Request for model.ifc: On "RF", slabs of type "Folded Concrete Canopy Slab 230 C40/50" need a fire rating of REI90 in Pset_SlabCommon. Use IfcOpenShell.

First a look at what the model holds.

```python
import ifcopenshell
import ifcopenshell.util.element

model = ifcopenshell.open("model.ifc")
print(model.schema)
storey = next(s for s in model.by_type("IfcBuildingStorey") if s.Name == "RF")
slabs = [e for e in ifcopenshell.util.element.get_decomposition(storey) if e.is_a("IfcSlab")]
seen = {}
for e in slabs:
    element_type = ifcopenshell.util.element.get_type(e)
    key = (element_type.Name if element_type != e and element_type else None, ifcopenshell.util.element.get_pset(e, "Pset_SlabCommon", "FireRating"))
    seen[key] = seen.get(key, 0) + 1
for (name, value), count in sorted(seen.items(), key=str):
    print(count, "x", name, "|", value)
```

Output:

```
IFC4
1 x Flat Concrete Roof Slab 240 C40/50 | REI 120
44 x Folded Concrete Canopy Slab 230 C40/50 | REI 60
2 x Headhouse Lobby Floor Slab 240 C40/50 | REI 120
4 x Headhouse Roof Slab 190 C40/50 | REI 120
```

```python
import ifcopenshell
import ifcopenshell.api.pset
import ifcopenshell.util.element

model = ifcopenshell.open("model.ifc")

storey = next(s for s in model.by_type("IfcBuildingStorey") if s.Name == "RF")
slabs = [e for e in ifcopenshell.util.element.get_decomposition(storey) if e.is_a("IfcSlab")]

count = 0
for e in slabs:
    element_type = ifcopenshell.util.element.get_type(e)
    if element_type in (None, e) or element_type.Name != "Folded Concrete Canopy Slab 230 C40/50":
        continue
    # add_pset returns the element's existing set when there is one.
    pset = ifcopenshell.api.pset.add_pset(model, product=e, name="Pset_SlabCommon")
    ifcopenshell.api.pset.edit_pset(model, pset=pset, properties={"FireRating": "REI90"})
    count += 1

print(count, "slabs updated")

model.write("model_v2.ifc")
```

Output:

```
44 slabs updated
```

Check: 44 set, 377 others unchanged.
